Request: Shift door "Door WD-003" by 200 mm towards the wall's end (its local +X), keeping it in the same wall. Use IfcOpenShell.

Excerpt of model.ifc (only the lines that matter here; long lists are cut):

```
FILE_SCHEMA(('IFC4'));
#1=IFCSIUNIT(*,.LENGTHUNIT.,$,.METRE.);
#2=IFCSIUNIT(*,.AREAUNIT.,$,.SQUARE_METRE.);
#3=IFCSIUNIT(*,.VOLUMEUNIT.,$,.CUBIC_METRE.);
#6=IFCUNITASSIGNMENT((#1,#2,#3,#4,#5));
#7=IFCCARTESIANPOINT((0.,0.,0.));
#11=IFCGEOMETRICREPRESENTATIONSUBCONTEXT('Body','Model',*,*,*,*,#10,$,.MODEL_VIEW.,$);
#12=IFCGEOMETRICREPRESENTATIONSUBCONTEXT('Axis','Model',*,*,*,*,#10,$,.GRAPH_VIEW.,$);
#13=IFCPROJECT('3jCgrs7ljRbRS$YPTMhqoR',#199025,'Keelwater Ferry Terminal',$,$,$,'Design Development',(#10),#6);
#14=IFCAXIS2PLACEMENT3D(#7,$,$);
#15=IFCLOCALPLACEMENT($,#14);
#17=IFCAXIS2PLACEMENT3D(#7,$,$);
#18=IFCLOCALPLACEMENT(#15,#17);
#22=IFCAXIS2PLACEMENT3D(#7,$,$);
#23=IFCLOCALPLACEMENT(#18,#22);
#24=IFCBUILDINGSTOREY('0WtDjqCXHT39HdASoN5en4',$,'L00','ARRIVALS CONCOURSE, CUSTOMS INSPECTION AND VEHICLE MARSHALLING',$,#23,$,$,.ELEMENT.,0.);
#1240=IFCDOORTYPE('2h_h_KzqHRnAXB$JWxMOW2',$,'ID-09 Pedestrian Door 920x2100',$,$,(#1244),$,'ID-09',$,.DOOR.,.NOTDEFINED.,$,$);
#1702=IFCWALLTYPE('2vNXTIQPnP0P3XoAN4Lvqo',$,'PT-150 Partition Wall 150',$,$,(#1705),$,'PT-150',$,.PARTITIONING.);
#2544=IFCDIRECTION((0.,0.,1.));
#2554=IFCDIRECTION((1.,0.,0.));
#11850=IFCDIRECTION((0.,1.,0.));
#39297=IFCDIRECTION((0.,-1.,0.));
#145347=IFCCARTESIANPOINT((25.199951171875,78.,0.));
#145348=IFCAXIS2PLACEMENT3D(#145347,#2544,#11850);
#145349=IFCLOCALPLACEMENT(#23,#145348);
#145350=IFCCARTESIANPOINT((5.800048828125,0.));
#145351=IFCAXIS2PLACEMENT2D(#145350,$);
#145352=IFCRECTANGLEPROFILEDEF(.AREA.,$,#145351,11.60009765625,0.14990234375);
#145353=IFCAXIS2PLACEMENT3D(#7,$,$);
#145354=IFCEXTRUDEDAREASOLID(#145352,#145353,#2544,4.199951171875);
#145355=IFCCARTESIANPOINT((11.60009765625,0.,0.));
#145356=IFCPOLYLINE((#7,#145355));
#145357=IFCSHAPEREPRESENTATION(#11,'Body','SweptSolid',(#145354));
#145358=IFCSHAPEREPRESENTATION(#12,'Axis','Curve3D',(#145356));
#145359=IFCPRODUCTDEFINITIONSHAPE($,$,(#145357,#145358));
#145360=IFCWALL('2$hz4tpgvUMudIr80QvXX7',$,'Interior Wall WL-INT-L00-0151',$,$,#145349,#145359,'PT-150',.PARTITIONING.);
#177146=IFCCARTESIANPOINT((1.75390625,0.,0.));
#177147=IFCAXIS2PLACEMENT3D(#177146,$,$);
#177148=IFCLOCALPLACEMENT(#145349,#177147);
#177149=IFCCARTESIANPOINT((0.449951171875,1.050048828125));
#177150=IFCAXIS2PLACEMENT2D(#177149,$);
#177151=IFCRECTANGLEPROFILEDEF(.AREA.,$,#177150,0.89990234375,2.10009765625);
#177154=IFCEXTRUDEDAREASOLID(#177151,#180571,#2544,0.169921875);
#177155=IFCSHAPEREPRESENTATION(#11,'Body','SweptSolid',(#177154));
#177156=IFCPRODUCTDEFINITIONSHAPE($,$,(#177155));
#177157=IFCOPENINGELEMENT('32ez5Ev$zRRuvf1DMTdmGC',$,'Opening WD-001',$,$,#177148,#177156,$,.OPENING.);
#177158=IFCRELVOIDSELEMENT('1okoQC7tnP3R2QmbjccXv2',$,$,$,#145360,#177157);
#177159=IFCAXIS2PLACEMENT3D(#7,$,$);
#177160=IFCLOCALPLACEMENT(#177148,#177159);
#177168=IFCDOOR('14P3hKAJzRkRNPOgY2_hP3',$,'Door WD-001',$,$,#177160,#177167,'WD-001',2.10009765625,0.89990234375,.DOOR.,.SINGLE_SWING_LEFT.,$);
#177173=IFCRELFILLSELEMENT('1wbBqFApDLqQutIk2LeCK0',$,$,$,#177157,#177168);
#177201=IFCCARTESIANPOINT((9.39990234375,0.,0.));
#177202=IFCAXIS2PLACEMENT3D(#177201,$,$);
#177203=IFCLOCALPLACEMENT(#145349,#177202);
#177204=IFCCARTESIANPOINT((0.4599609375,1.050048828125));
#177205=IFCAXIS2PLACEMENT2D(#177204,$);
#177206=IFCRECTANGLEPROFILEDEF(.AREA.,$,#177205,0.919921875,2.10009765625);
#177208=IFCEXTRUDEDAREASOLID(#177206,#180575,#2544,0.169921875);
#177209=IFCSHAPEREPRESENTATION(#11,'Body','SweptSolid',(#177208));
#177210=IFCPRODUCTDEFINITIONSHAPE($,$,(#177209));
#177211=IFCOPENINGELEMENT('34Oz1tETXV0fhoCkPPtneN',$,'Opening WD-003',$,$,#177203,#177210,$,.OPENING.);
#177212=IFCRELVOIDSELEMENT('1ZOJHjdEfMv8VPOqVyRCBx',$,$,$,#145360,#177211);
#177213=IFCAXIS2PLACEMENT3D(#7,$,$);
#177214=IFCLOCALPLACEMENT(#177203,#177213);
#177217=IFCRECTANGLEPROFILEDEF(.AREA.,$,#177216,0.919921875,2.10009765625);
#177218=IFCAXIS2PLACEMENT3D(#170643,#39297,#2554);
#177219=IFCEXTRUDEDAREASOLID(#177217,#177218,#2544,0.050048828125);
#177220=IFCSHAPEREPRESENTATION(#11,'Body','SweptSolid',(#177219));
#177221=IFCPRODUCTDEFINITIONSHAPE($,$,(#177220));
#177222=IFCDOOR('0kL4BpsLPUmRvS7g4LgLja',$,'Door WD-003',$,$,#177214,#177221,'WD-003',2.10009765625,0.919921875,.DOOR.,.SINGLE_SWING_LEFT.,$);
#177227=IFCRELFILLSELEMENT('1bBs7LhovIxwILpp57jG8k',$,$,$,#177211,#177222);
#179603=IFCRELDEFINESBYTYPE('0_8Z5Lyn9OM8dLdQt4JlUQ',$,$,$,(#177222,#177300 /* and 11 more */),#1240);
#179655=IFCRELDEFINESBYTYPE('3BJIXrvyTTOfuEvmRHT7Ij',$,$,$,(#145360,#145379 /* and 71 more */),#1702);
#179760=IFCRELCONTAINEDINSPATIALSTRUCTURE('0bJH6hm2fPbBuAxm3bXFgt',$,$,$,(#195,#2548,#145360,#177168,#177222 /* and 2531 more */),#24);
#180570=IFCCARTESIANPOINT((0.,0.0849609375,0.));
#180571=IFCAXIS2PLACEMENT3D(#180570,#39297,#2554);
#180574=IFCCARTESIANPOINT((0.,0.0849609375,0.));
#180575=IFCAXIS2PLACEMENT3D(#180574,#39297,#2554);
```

```python
import ifcopenshell
import ifcopenshell.api.geometry
import ifcopenshell.util.placement

model = ifcopenshell.open("model.ifc")

door = model.by_guid("0kL4BpsLPUmRvS7g4LgLja")
opening = door.FillsVoids[0].RelatingOpeningElement
wall = opening.VoidsElements[0].RelatingBuildingElement

wall_matrix = ifcopenshell.util.placement.get_local_placement(wall.ObjectPlacement)
shift = wall_matrix[:3, 0] * 0.2
before = ifcopenshell.util.placement.get_local_placement(door.ObjectPlacement)[:3, 3].copy()

# The door is placed relative to its opening, so it follows when the opening moves.
matrix = ifcopenshell.util.placement.get_local_placement(opening.ObjectPlacement)
matrix[:3, 3] += shift
ifcopenshell.api.geometry.edit_object_placement(
    model, product=opening, matrix=matrix, is_si=False, should_transform_children=True
)

after = ifcopenshell.util.placement.get_local_placement(door.ObjectPlacement)[:3, 3]
print("door moved by", (after - before).round(3) + 0.0)

model.write("model_rev.ifc")
```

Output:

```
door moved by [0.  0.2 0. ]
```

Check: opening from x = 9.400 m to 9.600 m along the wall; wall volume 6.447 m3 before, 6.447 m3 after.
